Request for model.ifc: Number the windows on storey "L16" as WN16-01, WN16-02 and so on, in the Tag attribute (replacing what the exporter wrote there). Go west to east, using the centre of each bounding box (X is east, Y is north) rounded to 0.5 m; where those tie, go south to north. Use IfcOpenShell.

First a look at what the model holds.

```python
import ifcopenshell
import ifcopenshell.util.element
import ifcopenshell.util.placement

model = ifcopenshell.open("model.ifc")
print(model.schema)
storey = next(s for s in model.by_type("IfcBuildingStorey") if s.Name == "L16")
windows = [e for e in ifcopenshell.util.element.get_decomposition(storey) if e.is_a("IfcWindow")]
for e in sorted(windows, key=lambda e: e.id()):
    origin = ifcopenshell.util.placement.get_local_placement(e.ObjectPlacement)[:3, 3]
    print(e.id(), e.Tag, e.Name, origin.round(2) + 0.0, sep=" | ")
```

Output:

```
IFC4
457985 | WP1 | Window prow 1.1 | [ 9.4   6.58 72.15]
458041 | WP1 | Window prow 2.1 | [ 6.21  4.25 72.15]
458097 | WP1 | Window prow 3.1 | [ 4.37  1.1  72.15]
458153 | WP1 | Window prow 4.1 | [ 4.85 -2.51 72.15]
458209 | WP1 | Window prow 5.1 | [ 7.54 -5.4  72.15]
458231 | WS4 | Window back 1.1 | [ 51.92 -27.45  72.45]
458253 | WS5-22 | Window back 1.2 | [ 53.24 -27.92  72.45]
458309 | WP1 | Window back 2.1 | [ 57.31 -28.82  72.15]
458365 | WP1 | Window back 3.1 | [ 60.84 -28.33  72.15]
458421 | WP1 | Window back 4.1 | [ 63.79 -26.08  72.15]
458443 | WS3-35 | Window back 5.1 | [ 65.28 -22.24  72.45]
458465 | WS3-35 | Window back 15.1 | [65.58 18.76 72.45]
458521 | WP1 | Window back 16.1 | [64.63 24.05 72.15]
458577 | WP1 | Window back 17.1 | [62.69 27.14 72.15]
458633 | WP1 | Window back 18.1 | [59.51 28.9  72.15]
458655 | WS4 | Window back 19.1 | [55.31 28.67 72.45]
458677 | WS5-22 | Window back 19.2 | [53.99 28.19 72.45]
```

```python
import ifcopenshell
import ifcopenshell.geom
import ifcopenshell.util.element
import ifcopenshell.util.shape

model = ifcopenshell.open("model.ifc")
settings = ifcopenshell.geom.settings()
settings.set("use-world-coords", True)


def centre(element):
    shape = ifcopenshell.geom.create_shape(settings, element)
    return ifcopenshell.util.shape.get_bbox_centroid(shape.geometry)


storey = next(s for s in model.by_type("IfcBuildingStorey") if s.Name == "L16")
windows = [e for e in ifcopenshell.util.element.get_decomposition(storey) if e.is_a("IfcWindow")]

# Insertion points can sit at a corner or the storey origin, so sort by the geometry (in metres).
centres = {e: centre(e) for e in windows}
windows.sort(key=lambda e: (round(centres[e][0] / 0.5), centres[e][1]))

for i, e in enumerate(windows, start=1):
    number = f"WN16-{i:02d}"
    e.Tag = number
    print(e.id(), number)

model.write("model_rev.ifc")
```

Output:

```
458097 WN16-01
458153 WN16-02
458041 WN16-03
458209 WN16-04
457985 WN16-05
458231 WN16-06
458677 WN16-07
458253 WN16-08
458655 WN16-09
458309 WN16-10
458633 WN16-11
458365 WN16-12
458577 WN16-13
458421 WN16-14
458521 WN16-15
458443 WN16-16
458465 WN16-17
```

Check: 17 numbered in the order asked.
